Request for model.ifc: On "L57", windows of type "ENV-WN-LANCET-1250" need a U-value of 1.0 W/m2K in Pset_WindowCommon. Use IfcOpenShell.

First a look at what the model holds.

```python
import ifcopenshell
import ifcopenshell.util.element

model = ifcopenshell.open("model.ifc")
print(model.schema)
storey = next(s for s in model.by_type("IfcBuildingStorey") if s.Name == "L57")
windows = [e for e in ifcopenshell.util.element.get_decomposition(storey) if e.is_a("IfcWindow")]
seen = {}
for e in windows:
    element_type = ifcopenshell.util.element.get_type(e)
    key = (element_type.Name if element_type != e and element_type else None, ifcopenshell.util.element.get_pset(e, "Pset_WindowCommon", "ThermalTransmittance"))
    seen[key] = seen.get(key, 0) + 1
for (name, value), count in sorted(seen.items(), key=str):
    print(count, "x", name, "|", value)
```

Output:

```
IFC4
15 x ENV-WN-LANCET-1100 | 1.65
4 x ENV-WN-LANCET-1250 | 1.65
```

```python
import ifcopenshell
import ifcopenshell.api.pset
import ifcopenshell.util.element

model = ifcopenshell.open("model.ifc")

storey = next(s for s in model.by_type("IfcBuildingStorey") if s.Name == "L57")
windows = [e for e in ifcopenshell.util.element.get_decomposition(storey) if e.is_a("IfcWindow")]

count = 0
for e in windows:
    element_type = ifcopenshell.util.element.get_type(e)
    if element_type in (None, e) or element_type.Name != "ENV-WN-LANCET-1250":
        continue
    # add_pset returns the element's existing set when there is one.
    pset = ifcopenshell.api.pset.add_pset(model, product=e, name="Pset_WindowCommon")
    ifcopenshell.api.pset.edit_pset(model, pset=pset, properties={"ThermalTransmittance": 1.0})
    count += 1

print(count, "windows updated")

model.write("model_v2.ifc")
```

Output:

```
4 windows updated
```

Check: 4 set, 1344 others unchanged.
